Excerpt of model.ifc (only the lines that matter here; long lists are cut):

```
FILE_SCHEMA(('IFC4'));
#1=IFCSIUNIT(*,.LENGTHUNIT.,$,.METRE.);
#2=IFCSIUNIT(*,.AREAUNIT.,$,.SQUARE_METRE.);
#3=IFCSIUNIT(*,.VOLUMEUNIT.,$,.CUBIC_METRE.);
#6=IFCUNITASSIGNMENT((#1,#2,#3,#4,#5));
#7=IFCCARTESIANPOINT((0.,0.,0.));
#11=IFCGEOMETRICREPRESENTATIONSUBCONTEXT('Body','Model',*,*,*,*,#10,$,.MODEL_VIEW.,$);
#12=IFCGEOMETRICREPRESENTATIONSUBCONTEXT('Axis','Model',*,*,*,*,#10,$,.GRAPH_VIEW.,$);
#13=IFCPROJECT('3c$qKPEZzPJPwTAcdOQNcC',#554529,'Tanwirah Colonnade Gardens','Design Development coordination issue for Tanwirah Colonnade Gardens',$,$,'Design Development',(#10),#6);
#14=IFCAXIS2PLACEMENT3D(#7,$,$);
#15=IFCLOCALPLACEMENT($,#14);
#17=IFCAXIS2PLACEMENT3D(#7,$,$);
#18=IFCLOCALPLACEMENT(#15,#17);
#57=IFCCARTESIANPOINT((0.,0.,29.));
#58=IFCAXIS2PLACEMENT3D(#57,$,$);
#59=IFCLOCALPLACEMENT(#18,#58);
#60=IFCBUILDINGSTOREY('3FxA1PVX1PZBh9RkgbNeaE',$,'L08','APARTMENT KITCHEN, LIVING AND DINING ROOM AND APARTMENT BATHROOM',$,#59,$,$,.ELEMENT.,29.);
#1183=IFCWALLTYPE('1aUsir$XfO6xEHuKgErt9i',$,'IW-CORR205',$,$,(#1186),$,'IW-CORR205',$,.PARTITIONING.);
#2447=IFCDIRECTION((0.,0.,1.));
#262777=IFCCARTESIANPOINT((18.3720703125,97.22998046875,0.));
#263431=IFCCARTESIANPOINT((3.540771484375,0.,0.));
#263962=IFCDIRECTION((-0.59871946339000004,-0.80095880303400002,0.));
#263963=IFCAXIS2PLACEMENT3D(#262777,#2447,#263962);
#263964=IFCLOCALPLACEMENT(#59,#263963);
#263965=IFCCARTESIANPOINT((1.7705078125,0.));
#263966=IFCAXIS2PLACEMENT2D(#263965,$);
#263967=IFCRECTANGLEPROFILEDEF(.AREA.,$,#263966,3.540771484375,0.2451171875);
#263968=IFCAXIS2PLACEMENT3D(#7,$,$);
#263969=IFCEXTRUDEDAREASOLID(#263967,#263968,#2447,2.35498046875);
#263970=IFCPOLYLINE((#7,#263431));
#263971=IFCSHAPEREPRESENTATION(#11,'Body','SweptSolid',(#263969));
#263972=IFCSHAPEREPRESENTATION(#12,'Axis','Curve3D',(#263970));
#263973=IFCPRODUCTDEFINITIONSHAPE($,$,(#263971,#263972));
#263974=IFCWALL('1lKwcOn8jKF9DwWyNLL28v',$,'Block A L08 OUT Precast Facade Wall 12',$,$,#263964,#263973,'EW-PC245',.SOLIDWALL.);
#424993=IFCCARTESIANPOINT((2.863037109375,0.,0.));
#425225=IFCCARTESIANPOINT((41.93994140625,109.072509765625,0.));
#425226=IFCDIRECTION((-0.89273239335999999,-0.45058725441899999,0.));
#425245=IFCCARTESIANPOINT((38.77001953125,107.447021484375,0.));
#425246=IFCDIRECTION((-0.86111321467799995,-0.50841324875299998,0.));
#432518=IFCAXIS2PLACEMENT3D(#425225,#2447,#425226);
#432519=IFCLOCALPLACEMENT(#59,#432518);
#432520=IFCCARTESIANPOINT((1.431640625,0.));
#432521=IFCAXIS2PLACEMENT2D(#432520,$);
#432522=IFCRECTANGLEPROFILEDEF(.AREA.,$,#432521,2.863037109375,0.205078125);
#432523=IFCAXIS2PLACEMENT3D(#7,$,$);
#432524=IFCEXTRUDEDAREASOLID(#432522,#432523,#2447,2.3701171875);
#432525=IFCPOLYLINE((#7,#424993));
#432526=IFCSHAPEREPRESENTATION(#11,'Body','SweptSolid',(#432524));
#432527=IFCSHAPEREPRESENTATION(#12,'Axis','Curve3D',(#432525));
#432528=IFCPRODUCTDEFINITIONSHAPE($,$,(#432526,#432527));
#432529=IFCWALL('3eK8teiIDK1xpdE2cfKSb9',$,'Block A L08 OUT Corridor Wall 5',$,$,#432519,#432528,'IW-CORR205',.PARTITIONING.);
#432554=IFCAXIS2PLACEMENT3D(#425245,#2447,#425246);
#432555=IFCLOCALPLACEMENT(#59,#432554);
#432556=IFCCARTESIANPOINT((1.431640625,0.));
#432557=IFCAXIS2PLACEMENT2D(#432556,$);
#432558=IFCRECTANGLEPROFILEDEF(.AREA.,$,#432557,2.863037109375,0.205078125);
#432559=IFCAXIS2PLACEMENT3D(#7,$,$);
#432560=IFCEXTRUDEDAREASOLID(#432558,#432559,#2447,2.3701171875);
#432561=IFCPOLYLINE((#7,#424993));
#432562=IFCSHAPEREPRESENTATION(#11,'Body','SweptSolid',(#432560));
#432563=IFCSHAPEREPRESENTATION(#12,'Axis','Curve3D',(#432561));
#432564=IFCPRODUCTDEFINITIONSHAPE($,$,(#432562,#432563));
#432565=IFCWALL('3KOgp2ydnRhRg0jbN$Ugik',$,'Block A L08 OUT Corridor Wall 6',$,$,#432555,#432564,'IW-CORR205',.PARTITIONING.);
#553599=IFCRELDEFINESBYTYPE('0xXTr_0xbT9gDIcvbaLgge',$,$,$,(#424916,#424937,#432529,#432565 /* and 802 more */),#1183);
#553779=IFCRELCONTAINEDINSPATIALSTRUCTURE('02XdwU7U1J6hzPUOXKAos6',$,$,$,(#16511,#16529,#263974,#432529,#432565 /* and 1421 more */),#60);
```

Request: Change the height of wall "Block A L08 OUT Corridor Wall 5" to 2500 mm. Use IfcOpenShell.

```python
import ifcopenshell
import ifcopenshell.geom
import ifcopenshell.util.representation
import ifcopenshell.util.shape

model = ifcopenshell.open("model.ifc")
settings = ifcopenshell.geom.settings()


def volume(element):
    """Net volume in cubic metres, openings subtracted."""
    shape = ifcopenshell.geom.create_shape(settings, element)
    return ifcopenshell.util.shape.get_volume(shape.geometry)


wall = model.by_guid("3eK8teiIDK1xpdE2cfKSb9")
before = volume(wall)

body = ifcopenshell.util.representation.get_representation(wall, "Model", "Body")
solid = body.Items[0]
old_height = solid.Depth
solid.Depth = 2.5
after = volume(wall)

print(f"height {old_height:g} -> {solid.Depth:g}, volume {before:.3f} -> {after:.3f} m3")

model.write("model_rev.ifc")
```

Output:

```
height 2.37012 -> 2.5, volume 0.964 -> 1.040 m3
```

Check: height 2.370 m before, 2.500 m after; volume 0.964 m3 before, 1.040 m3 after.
